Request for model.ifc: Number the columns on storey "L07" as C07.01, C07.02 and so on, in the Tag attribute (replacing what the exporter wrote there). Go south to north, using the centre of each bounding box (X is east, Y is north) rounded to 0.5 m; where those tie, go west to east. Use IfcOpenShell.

First a look at what the model holds.

```python
import ifcopenshell
import ifcopenshell.util.element
import ifcopenshell.util.placement

model = ifcopenshell.open("model.ifc")
print(model.schema)
storey = next(s for s in model.by_type("IfcBuildingStorey") if s.Name == "L07")
columns = [e for e in ifcopenshell.util.element.get_decomposition(storey) if e.is_a("IfcColumn")]
for e in sorted(columns, key=lambda e: e.id()):
    origin = ifcopenshell.util.placement.get_local_placement(e.ObjectPlacement)[:3, 3]
    print(e.id(), e.Tag, e.Name, origin.round(2) + 0.0, sep=" | ")
```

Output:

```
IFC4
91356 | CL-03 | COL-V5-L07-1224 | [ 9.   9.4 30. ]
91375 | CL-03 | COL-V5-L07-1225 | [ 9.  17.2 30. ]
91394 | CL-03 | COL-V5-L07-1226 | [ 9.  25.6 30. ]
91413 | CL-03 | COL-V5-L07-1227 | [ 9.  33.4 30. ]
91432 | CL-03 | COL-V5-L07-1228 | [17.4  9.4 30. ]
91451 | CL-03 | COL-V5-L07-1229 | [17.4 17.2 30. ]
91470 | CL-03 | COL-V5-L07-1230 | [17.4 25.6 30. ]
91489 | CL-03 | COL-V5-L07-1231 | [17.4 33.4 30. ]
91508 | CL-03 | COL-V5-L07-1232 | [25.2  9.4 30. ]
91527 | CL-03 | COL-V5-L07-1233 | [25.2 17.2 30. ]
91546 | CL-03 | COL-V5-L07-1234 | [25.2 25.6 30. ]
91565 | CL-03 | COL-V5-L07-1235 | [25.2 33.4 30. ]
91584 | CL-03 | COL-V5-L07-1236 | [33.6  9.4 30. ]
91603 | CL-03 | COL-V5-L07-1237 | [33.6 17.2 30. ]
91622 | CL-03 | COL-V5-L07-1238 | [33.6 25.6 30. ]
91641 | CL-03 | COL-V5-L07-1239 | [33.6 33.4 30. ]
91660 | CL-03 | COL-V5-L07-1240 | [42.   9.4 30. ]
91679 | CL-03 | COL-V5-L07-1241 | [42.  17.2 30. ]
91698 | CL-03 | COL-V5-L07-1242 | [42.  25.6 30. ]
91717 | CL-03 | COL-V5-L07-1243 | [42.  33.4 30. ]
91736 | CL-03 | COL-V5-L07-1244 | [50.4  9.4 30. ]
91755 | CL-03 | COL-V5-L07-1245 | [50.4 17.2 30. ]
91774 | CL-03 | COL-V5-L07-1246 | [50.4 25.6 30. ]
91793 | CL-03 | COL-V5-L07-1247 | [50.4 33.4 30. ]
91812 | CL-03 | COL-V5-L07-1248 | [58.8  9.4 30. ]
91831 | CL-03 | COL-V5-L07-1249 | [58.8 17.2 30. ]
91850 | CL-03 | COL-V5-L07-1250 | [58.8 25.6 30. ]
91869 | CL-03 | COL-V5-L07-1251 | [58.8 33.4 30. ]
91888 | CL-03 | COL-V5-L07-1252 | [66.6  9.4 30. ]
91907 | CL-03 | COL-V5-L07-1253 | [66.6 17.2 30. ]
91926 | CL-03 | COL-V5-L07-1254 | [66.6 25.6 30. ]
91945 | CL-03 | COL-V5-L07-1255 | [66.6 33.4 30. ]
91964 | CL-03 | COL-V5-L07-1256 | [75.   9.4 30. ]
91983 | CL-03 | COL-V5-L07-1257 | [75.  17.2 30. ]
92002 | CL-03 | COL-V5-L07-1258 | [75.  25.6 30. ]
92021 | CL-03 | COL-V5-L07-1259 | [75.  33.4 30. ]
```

```python
import ifcopenshell
import ifcopenshell.geom
import ifcopenshell.util.element
import ifcopenshell.util.shape

model = ifcopenshell.open("model.ifc")
settings = ifcopenshell.geom.settings()
settings.set("use-world-coords", True)


def centre(element):
    shape = ifcopenshell.geom.create_shape(settings, element)
    return ifcopenshell.util.shape.get_bbox_centroid(shape.geometry)


storey = next(s for s in model.by_type("IfcBuildingStorey") if s.Name == "L07")
columns = [e for e in ifcopenshell.util.element.get_decomposition(storey) if e.is_a("IfcColumn")]

# Insertion points can sit at a corner or the storey origin, so sort by the geometry (in metres).
centres = {e: centre(e) for e in columns}
columns.sort(key=lambda e: (round(centres[e][1] / 0.5), centres[e][0]))

for i, e in enumerate(columns, start=1):
    number = f"C07.{i:02d}"
    e.Tag = number
    print(e.id(), number)

model.write("model_v2.ifc")
```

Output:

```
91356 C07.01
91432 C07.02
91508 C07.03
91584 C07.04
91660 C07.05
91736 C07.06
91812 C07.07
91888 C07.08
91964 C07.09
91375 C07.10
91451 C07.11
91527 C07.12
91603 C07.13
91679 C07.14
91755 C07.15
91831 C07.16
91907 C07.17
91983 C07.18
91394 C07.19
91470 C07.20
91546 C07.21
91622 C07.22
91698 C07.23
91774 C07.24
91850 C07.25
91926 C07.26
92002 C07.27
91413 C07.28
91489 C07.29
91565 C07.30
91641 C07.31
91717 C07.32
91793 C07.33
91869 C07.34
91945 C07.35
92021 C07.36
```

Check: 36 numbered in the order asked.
